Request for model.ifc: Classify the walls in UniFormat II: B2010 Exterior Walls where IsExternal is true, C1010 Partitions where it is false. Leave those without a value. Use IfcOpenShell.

First a look at what the model holds.

```python
import ifcopenshell
import ifcopenshell.util.element

model = ifcopenshell.open("model.ifc")
print(model.schema)
print("classifications:", [c.Name for c in model.by_type("IfcClassification")])
values = [ifcopenshell.util.element.get_pset(e, "Pset_WallCommon", "IsExternal") for e in model.by_type("IfcWall")]
for value in (True, False, None):
    print("IsExternal", value, values.count(value))
```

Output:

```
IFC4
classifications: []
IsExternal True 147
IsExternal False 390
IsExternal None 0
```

```python
import ifcopenshell
import ifcopenshell.api.classification
import ifcopenshell.util.element

model = ifcopenshell.open("model.ifc")

system = ifcopenshell.api.classification.add_classification(model, classification="UniFormat II")

walls = model.by_type("IfcWall")
external = {e: ifcopenshell.util.element.get_pset(e, "Pset_WallCommon", "IsExternal") for e in walls}
for flag, code, name in ((True, "B2010", "Exterior Walls"), (False, "C1010", "Partitions")):
    products = [e for e in walls if external[e] is flag]
    ifcopenshell.api.classification.add_reference(
        model, products=products, classification=system, identification=code, name=name
    )
    print(code, len(products))

model.write("model_edited.ifc")
```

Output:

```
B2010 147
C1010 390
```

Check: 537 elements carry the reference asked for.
